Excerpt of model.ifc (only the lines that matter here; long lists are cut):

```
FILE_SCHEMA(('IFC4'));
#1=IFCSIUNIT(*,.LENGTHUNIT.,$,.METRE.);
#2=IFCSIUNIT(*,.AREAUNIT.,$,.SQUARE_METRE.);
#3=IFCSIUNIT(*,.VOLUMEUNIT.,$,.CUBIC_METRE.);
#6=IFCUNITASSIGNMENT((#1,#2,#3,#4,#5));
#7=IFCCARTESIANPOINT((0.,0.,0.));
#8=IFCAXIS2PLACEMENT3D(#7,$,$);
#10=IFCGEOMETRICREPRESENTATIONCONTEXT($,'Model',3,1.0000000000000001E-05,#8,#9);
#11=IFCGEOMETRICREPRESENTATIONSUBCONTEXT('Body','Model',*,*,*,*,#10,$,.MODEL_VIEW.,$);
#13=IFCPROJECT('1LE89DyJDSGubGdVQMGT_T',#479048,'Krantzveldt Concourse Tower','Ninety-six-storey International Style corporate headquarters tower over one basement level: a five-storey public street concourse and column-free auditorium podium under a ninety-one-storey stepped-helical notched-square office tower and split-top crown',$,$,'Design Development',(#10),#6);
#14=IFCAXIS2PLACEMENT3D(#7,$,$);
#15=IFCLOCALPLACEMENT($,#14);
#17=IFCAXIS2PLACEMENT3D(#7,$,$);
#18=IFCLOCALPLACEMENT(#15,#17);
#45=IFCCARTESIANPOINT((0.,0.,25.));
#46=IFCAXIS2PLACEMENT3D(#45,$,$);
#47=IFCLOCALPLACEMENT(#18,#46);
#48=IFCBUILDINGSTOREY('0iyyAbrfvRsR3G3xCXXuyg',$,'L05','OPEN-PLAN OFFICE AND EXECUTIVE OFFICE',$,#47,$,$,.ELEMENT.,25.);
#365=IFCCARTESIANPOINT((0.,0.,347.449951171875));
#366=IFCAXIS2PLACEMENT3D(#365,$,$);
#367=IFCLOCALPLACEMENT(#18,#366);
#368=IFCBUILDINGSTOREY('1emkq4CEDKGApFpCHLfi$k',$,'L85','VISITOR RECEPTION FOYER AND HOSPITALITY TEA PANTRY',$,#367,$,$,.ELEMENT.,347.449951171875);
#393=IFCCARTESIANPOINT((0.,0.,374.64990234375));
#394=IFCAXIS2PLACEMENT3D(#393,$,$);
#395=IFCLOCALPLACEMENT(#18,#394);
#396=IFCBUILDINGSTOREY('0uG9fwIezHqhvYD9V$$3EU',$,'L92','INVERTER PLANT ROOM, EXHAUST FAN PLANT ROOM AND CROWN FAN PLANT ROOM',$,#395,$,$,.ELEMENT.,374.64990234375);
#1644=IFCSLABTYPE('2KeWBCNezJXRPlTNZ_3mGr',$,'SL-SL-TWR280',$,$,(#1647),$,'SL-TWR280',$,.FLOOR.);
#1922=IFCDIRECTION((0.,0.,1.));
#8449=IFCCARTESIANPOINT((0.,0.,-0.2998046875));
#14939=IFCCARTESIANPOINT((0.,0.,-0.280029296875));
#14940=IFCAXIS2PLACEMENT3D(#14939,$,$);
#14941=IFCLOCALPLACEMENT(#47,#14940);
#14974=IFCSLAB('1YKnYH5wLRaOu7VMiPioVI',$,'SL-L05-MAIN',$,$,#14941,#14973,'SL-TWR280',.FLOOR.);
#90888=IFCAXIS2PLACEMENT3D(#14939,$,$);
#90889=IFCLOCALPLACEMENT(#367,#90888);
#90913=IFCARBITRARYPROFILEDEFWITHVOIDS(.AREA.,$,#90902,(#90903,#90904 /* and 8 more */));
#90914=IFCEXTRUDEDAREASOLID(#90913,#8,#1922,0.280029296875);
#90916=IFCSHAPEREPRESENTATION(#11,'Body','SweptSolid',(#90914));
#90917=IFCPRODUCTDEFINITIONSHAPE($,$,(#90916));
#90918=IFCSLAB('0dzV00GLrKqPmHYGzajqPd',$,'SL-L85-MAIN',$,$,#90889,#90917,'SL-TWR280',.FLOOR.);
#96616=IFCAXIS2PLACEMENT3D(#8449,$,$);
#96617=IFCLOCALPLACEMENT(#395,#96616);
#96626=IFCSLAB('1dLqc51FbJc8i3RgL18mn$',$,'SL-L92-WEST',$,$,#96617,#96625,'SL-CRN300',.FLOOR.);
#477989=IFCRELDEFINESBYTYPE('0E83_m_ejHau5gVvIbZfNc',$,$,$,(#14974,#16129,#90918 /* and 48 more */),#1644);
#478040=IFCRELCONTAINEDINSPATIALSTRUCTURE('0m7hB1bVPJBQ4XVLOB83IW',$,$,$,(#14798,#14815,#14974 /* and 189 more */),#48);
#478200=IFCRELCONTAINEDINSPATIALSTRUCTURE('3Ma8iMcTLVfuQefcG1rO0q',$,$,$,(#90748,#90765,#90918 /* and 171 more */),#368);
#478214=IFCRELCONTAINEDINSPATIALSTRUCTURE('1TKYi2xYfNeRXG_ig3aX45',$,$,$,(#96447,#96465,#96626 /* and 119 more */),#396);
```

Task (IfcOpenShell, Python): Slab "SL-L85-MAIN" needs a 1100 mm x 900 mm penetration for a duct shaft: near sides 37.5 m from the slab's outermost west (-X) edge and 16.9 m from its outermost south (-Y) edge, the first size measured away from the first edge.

```python
import numpy as np
import ifcopenshell
import ifcopenshell.api.feature
import ifcopenshell.api.geometry
import ifcopenshell.api.root
import ifcopenshell.geom
import ifcopenshell.util.placement
import ifcopenshell.util.representation
import ifcopenshell.util.shape
import ifcopenshell.util.unit

model = ifcopenshell.open("model.ifc")
unit_scale = ifcopenshell.util.unit.calculate_unit_scale(model)
settings = ifcopenshell.geom.settings()


def volume(element):
    """Net volume in cubic metres, openings subtracted."""
    shape = ifcopenshell.geom.create_shape(settings, element)
    return ifcopenshell.util.shape.get_volume(shape.geometry)


slab = model.by_guid("0dzV00GLrKqPmHYGzajqPd")
before = volume(slab)

# Extent in the slab's own axes, in metres. The edges named are its -X and -Y sides.
slab_shape = ifcopenshell.geom.create_shape(settings, slab)
vertices = ifcopenshell.util.shape.get_vertices(slab_shape.geometry)
x_min, y_min, bottom = vertices.min(axis=0)
top = vertices[:, 2].max()

opening = ifcopenshell.api.root.create_entity(model, ifc_class="IfcOpeningElement", name="Duct shaft opening", predefined_type="OPENING")
context = ifcopenshell.util.representation.get_context(model, "Model", "Body", "MODEL_VIEW")
width, depth = 1.1, 0.9
outline = [(0.0, 0.0), (width, 0.0), (width, depth), (0.0, depth), (0.0, 0.0)]
# Overshoot both faces by 50 mm so the cut is clean.
shape = ifcopenshell.api.geometry.add_slab_representation(
    model, context=context, depth=top - bottom + 0.1, polyline=outline
)
ifcopenshell.api.geometry.assign_representation(model, product=opening, representation=shape)

matrix = ifcopenshell.util.placement.get_local_placement(slab.ObjectPlacement)
matrix[:, 3] = matrix @ np.append(np.array([x_min + 37.5, y_min + 16.9, bottom - 0.05]) / unit_scale, 1.0)
ifcopenshell.api.geometry.edit_object_placement(model, product=opening, matrix=matrix, is_si=False)
ifcopenshell.api.feature.add_feature(model, feature=opening, element=slab)

after = volume(slab)

print(f"slab volume {before:.3f} -> {after:.3f} m3")

model.write("model_v2.ifc")
```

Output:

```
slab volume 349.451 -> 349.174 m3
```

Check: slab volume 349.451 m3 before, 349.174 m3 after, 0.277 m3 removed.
